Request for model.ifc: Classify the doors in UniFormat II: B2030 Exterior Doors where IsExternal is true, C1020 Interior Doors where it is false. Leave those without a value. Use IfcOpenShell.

First a look at what the model holds.

```python
import ifcopenshell
import ifcopenshell.util.element

model = ifcopenshell.open("model.ifc")
print(model.schema)
print("classifications:", [c.Name for c in model.by_type("IfcClassification")])
values = [ifcopenshell.util.element.get_pset(e, "Pset_DoorCommon", "IsExternal") for e in model.by_type("IfcDoor")]
for value in (True, False, None):
    print("IsExternal", value, values.count(value))
```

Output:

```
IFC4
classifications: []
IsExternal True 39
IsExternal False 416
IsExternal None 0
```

```python
import ifcopenshell
import ifcopenshell.api.classification
import ifcopenshell.util.element

model = ifcopenshell.open("model.ifc")

system = ifcopenshell.api.classification.add_classification(model, classification="UniFormat II")

doors = model.by_type("IfcDoor")
external = {e: ifcopenshell.util.element.get_pset(e, "Pset_DoorCommon", "IsExternal") for e in doors}
for flag, code, name in ((True, "B2030", "Exterior Doors"), (False, "C1020", "Interior Doors")):
    products = [e for e in doors if external[e] is flag]
    ifcopenshell.api.classification.add_reference(
        model, products=products, classification=system, identification=code, name=name
    )
    print(code, len(products))

model.write("model_v2.ifc")
```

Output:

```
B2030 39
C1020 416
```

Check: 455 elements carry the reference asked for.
